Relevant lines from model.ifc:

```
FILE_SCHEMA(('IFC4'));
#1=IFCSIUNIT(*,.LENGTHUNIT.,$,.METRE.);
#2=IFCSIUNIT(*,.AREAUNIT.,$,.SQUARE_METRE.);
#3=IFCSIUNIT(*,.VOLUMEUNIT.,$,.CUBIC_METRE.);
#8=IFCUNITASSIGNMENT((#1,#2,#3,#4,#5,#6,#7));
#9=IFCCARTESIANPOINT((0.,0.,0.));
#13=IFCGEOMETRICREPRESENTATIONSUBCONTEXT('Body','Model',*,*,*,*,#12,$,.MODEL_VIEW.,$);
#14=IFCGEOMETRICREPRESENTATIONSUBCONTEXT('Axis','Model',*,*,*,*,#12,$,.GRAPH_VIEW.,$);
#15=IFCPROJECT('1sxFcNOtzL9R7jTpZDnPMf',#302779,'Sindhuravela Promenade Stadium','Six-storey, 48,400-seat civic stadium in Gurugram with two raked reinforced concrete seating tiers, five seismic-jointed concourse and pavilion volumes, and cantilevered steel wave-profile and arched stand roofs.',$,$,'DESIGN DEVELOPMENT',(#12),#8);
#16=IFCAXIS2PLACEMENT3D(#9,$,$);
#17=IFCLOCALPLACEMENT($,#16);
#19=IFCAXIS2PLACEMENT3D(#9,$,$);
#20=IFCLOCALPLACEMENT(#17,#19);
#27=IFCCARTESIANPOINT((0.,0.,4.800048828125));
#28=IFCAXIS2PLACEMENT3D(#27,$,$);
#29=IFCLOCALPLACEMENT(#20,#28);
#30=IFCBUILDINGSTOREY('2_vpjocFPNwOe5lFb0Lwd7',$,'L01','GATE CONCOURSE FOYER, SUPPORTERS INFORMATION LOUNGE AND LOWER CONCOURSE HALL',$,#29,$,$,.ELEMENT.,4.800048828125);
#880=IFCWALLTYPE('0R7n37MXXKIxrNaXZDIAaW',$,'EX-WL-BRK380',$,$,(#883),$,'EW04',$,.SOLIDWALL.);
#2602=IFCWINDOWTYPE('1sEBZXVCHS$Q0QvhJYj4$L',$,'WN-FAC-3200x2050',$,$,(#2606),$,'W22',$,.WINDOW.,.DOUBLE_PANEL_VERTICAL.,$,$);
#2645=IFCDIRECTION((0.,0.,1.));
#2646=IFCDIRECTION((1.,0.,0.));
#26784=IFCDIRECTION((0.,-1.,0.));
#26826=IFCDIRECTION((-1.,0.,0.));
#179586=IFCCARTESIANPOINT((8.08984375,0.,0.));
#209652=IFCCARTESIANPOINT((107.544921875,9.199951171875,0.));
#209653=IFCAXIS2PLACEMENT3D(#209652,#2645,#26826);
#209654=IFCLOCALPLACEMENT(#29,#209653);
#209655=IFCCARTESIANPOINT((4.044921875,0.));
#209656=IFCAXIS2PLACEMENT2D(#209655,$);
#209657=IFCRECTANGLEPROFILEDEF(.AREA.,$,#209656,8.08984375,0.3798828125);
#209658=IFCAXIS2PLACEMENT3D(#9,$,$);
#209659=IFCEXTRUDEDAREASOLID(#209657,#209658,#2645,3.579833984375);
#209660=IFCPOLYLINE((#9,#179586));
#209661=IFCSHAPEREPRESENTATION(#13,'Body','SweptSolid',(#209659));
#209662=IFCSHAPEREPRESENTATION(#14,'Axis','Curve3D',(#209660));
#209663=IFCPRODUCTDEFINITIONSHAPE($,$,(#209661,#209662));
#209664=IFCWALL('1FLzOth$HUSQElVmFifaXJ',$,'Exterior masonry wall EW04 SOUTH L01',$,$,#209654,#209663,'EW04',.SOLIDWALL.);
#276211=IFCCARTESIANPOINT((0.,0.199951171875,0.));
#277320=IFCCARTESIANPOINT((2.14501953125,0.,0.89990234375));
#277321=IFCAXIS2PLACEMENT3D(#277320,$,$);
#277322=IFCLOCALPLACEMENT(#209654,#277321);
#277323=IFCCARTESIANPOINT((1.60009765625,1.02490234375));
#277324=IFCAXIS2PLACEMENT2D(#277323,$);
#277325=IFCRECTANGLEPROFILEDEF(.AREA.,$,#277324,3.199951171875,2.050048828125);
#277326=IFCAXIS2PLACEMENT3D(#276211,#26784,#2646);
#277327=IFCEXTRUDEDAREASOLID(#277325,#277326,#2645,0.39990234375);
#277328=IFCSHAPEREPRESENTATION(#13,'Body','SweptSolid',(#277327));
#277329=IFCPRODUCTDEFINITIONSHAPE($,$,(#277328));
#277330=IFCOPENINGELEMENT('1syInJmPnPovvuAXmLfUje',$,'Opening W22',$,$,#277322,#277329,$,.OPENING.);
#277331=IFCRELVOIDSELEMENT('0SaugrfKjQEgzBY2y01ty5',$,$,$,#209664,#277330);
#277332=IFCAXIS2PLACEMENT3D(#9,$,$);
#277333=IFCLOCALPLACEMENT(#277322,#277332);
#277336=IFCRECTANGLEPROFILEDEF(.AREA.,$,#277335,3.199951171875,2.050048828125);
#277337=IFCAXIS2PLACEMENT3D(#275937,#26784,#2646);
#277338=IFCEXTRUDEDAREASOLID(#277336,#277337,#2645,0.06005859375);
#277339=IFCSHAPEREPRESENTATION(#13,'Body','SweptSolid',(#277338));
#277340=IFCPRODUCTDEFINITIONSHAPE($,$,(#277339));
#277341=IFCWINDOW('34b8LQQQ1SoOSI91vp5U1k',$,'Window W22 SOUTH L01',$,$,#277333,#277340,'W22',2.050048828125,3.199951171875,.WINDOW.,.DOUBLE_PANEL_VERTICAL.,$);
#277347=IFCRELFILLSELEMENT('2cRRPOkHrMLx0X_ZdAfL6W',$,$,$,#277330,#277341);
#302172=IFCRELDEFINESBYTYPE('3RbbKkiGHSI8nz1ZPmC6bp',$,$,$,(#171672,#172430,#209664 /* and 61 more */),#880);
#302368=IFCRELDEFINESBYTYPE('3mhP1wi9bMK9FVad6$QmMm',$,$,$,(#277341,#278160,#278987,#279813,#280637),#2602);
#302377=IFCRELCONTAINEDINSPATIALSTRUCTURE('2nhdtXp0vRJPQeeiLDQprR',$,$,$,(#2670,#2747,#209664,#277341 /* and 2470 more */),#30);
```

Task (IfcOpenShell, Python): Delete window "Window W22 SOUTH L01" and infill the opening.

```python
import ifcopenshell
import ifcopenshell.api.feature
import ifcopenshell.api.root
import ifcopenshell.geom
import ifcopenshell.util.shape

model = ifcopenshell.open("model.ifc")
settings = ifcopenshell.geom.settings()


def volume(element):
    """Net volume in cubic metres, openings subtracted."""
    shape = ifcopenshell.geom.create_shape(settings, element)
    return ifcopenshell.util.shape.get_volume(shape.geometry)


window = model.by_guid("34b8LQQQ1SoOSI91vp5U1k")
opening = window.FillsVoids[0].RelatingOpeningElement
wall = opening.VoidsElements[0].RelatingBuildingElement
before = volume(wall)

ifcopenshell.api.root.remove_product(model, product=window)
ifcopenshell.api.feature.remove_feature(model, feature=opening)

after = volume(wall)

print(f"wall volume {before:.3f} -> {after:.3f} m3")

model.write("model_rev.ifc")
```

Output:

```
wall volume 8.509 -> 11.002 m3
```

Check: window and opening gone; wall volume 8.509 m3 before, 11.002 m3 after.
